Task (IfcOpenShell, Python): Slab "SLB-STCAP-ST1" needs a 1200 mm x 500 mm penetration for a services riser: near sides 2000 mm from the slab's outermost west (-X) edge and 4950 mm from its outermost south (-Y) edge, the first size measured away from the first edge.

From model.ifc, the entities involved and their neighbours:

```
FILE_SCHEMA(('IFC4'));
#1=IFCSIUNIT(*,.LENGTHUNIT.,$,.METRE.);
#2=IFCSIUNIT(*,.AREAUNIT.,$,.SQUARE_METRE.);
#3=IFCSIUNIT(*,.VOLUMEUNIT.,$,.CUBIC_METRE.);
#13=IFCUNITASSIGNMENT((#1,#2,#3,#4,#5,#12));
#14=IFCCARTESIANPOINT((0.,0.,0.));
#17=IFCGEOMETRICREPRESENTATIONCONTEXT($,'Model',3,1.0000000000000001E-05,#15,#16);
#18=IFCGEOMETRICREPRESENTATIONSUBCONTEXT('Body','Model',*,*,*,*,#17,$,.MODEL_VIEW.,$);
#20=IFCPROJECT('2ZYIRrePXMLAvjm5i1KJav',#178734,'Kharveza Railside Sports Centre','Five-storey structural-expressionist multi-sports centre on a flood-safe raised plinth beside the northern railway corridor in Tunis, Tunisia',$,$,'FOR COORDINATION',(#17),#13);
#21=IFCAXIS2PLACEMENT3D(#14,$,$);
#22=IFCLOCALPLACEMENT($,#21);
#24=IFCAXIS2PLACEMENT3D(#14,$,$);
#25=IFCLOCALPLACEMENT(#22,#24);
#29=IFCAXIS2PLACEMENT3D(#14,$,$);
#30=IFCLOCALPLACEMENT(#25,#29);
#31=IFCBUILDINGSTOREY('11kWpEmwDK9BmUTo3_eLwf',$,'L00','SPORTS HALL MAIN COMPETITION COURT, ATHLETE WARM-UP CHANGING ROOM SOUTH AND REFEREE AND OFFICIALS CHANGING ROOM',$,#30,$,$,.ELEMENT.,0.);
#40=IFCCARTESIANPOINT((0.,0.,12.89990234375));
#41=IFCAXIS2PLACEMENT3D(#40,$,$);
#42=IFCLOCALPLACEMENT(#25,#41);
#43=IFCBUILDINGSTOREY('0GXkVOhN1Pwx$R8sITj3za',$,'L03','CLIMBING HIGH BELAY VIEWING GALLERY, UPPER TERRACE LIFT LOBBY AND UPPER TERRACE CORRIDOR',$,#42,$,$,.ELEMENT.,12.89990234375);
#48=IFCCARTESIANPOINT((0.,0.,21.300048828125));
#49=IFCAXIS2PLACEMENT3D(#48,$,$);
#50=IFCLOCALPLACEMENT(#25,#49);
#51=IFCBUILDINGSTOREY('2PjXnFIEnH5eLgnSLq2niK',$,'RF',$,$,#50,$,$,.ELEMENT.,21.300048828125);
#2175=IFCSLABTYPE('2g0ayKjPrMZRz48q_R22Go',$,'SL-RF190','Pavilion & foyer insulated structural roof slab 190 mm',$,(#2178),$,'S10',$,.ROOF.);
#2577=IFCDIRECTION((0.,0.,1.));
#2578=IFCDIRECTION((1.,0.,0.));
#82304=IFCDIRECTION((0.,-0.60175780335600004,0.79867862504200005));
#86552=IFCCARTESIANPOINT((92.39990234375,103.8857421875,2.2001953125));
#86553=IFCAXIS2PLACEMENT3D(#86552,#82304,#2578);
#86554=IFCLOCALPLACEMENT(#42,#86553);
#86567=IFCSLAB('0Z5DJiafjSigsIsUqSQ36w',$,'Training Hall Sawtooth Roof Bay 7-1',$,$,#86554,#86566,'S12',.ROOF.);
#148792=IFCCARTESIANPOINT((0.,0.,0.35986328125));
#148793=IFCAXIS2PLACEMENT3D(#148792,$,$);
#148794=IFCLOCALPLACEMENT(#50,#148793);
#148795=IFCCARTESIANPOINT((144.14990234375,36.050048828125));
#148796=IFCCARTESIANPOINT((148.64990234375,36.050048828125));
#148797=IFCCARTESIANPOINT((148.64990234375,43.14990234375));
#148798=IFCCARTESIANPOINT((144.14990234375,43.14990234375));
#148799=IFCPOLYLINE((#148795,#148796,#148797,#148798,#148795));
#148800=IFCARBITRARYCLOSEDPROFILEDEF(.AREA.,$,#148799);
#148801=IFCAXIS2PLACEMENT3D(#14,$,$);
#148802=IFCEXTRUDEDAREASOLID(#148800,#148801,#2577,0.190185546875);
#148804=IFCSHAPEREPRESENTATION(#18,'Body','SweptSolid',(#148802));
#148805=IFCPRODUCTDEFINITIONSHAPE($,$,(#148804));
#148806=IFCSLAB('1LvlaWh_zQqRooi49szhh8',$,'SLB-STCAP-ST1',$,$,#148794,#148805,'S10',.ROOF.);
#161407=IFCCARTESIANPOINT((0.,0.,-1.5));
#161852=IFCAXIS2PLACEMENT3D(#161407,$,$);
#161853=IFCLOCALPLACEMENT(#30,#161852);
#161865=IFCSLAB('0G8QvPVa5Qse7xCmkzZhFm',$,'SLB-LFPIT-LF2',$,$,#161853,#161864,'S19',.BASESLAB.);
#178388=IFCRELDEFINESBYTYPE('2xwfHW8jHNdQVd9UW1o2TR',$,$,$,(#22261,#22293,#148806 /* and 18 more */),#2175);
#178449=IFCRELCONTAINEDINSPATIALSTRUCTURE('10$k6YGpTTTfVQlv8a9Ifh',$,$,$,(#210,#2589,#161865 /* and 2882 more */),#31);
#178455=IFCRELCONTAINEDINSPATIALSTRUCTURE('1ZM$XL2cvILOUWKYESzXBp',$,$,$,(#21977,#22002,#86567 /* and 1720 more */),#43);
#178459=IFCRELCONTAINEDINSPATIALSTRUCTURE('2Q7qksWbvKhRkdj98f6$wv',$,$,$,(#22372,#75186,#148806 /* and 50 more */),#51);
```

```python
import numpy as np
import ifcopenshell
import ifcopenshell.api.feature
import ifcopenshell.api.geometry
import ifcopenshell.api.root
import ifcopenshell.geom
import ifcopenshell.util.placement
import ifcopenshell.util.representation
import ifcopenshell.util.shape
import ifcopenshell.util.unit

model = ifcopenshell.open("model.ifc")
unit_scale = ifcopenshell.util.unit.calculate_unit_scale(model)
settings = ifcopenshell.geom.settings()


def volume(element):
    """Net volume in cubic metres, openings subtracted."""
    shape = ifcopenshell.geom.create_shape(settings, element)
    return ifcopenshell.util.shape.get_volume(shape.geometry)


slab = model.by_id(148806)
before = volume(slab)

# Extent in the slab's own axes, in metres. The edges named are its -X and -Y sides.
slab_shape = ifcopenshell.geom.create_shape(settings, slab)
vertices = ifcopenshell.util.shape.get_vertices(slab_shape.geometry)
x_min, y_min, bottom = vertices.min(axis=0)
top = vertices[:, 2].max()

opening = ifcopenshell.api.root.create_entity(model, ifc_class="IfcOpeningElement", name="Services riser opening", predefined_type="OPENING")
context = ifcopenshell.util.representation.get_context(model, "Model", "Body", "MODEL_VIEW")
width, depth = 1.2, 0.5
outline = [(0.0, 0.0), (width, 0.0), (width, depth), (0.0, depth), (0.0, 0.0)]
# Overshoot both faces by 50 mm so the cut is clean.
shape = ifcopenshell.api.geometry.add_slab_representation(
    model, context=context, depth=top - bottom + 0.1, polyline=outline
)
ifcopenshell.api.geometry.assign_representation(model, product=opening, representation=shape)

matrix = ifcopenshell.util.placement.get_local_placement(slab.ObjectPlacement)
matrix[:, 3] = matrix @ np.append(np.array([x_min + 2, y_min + 4.95, bottom - 0.05]) / unit_scale, 1.0)
ifcopenshell.api.geometry.edit_object_placement(model, product=opening, matrix=matrix, is_si=False)
ifcopenshell.api.feature.add_feature(model, feature=opening, element=slab)

after = volume(slab)

print(f"slab volume {before:.3f} -> {after:.3f} m3")

model.write("model-out.ifc")
```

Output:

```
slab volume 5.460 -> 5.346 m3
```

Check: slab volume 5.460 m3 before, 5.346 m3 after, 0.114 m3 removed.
